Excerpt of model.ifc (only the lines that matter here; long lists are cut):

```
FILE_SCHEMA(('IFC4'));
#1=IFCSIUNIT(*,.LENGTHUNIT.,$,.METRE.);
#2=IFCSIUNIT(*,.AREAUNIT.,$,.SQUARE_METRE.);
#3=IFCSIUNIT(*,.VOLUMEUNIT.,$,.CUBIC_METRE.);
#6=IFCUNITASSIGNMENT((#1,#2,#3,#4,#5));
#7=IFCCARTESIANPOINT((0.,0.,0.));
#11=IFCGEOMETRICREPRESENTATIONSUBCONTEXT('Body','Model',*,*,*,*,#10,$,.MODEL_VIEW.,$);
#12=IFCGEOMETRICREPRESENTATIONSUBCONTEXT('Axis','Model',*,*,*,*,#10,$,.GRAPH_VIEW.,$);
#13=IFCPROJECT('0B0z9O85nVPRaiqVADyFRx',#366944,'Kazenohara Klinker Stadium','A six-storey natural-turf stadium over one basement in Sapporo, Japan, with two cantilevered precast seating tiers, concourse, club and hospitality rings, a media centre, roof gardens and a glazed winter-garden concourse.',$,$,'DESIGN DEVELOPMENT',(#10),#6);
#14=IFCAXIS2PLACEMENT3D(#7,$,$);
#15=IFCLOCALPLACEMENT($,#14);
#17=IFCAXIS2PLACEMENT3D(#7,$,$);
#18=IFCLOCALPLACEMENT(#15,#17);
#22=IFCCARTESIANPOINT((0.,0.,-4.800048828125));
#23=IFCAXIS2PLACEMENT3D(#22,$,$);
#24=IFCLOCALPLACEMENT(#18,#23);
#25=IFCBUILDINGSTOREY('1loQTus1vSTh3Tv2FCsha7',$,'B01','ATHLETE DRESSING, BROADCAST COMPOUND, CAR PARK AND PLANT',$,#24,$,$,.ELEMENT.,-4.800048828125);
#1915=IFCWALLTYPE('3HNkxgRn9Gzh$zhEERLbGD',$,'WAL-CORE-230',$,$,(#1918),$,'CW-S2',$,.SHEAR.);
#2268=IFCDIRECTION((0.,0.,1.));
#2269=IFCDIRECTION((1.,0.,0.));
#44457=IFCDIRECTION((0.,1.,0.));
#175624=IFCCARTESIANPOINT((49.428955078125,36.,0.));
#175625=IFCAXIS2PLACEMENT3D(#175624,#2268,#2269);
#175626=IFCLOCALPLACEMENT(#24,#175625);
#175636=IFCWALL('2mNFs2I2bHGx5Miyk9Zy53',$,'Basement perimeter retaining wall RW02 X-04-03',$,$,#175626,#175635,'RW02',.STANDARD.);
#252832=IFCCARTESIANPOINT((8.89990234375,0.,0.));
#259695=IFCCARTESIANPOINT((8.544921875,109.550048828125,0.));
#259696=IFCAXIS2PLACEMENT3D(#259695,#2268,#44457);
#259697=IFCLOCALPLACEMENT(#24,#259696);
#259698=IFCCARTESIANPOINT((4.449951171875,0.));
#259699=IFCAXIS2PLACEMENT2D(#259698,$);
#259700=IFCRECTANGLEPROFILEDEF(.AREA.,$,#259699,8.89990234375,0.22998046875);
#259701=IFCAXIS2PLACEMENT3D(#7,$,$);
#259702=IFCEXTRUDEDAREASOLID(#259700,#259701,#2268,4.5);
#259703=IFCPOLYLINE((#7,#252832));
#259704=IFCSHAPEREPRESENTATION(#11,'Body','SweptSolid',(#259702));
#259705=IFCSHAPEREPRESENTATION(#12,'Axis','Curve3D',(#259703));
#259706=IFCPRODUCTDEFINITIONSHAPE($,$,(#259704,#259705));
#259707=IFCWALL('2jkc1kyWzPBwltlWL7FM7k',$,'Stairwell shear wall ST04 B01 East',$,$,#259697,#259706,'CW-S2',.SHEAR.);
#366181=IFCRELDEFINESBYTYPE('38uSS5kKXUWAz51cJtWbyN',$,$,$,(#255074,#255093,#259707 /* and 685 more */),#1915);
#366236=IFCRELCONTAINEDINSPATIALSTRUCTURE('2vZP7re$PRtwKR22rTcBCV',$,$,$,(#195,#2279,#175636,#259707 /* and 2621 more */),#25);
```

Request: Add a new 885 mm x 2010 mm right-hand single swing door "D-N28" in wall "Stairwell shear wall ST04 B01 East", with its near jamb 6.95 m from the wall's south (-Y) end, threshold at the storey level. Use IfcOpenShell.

```python
import numpy as np
import ifcopenshell
import ifcopenshell.api.feature
import ifcopenshell.api.geometry
import ifcopenshell.api.root
import ifcopenshell.api.spatial
import ifcopenshell.geom
import ifcopenshell.util.element
import ifcopenshell.util.placement
import ifcopenshell.util.representation
import ifcopenshell.util.shape
import ifcopenshell.util.unit

model = ifcopenshell.open("model.ifc")
unit_scale = ifcopenshell.util.unit.calculate_unit_scale(model)
settings = ifcopenshell.geom.settings()


def volume(element):
    """Net volume in cubic metres, openings subtracted."""
    shape = ifcopenshell.geom.create_shape(settings, element)
    return ifcopenshell.util.shape.get_volume(shape.geometry)


wall = model.by_id(259707)
storey = ifcopenshell.util.element.get_container(wall, ifc_class="IfcBuildingStorey")
context = ifcopenshell.util.representation.get_context(model, "Model", "Body", "MODEL_VIEW")
before = volume(wall)

width, height, from_end, sill = 0.885, 2.01, 6.95, 0.0  # metres

# The wall runs along its own X axis, and the end named is its -X end.
wall_shape = ifcopenshell.geom.create_shape(settings, wall)
x, y, z = ifcopenshell.util.shape.get_vertices(wall_shape.geometry).T
start = x.min() + from_end
face, thickness = float(y.min()), float(y.max() - y.min())
wall_matrix = ifcopenshell.util.placement.get_local_placement(wall.ObjectPlacement)
level = ifcopenshell.util.placement.get_local_placement(storey.ObjectPlacement)[2, 3]


def in_wall(x, y):
    """Placement at x, y metres in the wall's axes, at sill height."""
    matrix = wall_matrix.copy()
    matrix[:, 3] = wall_matrix @ np.array([x / unit_scale, y / unit_scale, 0.0, 1.0])
    matrix[2, 3] = level + sill / unit_scale
    return matrix


# Opening: a box that overshoots both wall faces by 50 mm.
opening = ifcopenshell.api.root.create_entity(model, ifc_class="IfcOpeningElement", predefined_type="OPENING")
box = ifcopenshell.api.geometry.add_wall_representation(
    model, context=context, length=width, height=height, thickness=thickness + 0.1
)
ifcopenshell.api.geometry.assign_representation(model, product=opening, representation=box)
ifcopenshell.api.geometry.edit_object_placement(model, product=opening, matrix=in_wall(start, face - 0.05), is_si=False)
ifcopenshell.api.feature.add_feature(model, feature=opening, element=wall)

door = ifcopenshell.api.root.create_entity(model, ifc_class="IfcDoor", name="D-N28", predefined_type="DOOR")
door.OverallWidth, door.OverallHeight = width / unit_scale, height / unit_scale
door.OperationType = "SINGLE_SWING_RIGHT"
body = ifcopenshell.api.geometry.add_door_representation(
    model,
    context=context,
    overall_width=door.OverallWidth,
    overall_height=door.OverallHeight,
    operation_type="SINGLE_SWING_RIGHT",
    lining_properties={"LiningDepth": thickness / unit_scale, "ThresholdDepth": thickness / unit_scale},
)
ifcopenshell.api.geometry.assign_representation(model, product=door, representation=body)
ifcopenshell.api.spatial.assign_container(model, products=[door], relating_structure=storey)
ifcopenshell.api.feature.add_filling(model, opening=opening, element=door)

# The lining spans the wall, so the door starts at the wall face.
ifcopenshell.api.geometry.edit_object_placement(model, product=door, matrix=in_wall(start, face), is_si=False)

after = volume(wall)

print(f"wall volume {before:.3f} -> {after:.3f} m3")

model.write("model_updated.ifc")
```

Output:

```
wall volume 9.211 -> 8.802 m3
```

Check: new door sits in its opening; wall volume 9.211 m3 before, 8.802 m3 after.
